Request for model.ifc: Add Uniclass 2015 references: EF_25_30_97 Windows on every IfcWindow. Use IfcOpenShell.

First a look at what the model holds.

```python
import ifcopenshell

model = ifcopenshell.open("model.ifc")
print(model.schema)
print("classifications:", [c.Name for c in model.by_type("IfcClassification")])
for ifc_class in ("IfcDoor", "IfcRoof", "IfcStair", "IfcWall", "IfcWindow"):
    print(ifc_class, len(model.by_type(ifc_class)))
```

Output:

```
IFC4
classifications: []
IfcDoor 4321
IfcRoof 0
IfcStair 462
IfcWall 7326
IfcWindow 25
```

```python
import ifcopenshell
import ifcopenshell.api.classification

model = ifcopenshell.open("model.ifc")

system = ifcopenshell.api.classification.add_classification(model, classification="Uniclass 2015")

codes = {
    "IfcWindow": ("EF_25_30_97", "Windows"),
}
for ifc_class, (code, name) in codes.items():
    products = model.by_type(ifc_class)
    ifcopenshell.api.classification.add_reference(
        model, products=products, classification=system, identification=code, name=name
    )
    print(code, len(products))

model.write("model_edited.ifc")
```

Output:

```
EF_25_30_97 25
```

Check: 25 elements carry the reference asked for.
